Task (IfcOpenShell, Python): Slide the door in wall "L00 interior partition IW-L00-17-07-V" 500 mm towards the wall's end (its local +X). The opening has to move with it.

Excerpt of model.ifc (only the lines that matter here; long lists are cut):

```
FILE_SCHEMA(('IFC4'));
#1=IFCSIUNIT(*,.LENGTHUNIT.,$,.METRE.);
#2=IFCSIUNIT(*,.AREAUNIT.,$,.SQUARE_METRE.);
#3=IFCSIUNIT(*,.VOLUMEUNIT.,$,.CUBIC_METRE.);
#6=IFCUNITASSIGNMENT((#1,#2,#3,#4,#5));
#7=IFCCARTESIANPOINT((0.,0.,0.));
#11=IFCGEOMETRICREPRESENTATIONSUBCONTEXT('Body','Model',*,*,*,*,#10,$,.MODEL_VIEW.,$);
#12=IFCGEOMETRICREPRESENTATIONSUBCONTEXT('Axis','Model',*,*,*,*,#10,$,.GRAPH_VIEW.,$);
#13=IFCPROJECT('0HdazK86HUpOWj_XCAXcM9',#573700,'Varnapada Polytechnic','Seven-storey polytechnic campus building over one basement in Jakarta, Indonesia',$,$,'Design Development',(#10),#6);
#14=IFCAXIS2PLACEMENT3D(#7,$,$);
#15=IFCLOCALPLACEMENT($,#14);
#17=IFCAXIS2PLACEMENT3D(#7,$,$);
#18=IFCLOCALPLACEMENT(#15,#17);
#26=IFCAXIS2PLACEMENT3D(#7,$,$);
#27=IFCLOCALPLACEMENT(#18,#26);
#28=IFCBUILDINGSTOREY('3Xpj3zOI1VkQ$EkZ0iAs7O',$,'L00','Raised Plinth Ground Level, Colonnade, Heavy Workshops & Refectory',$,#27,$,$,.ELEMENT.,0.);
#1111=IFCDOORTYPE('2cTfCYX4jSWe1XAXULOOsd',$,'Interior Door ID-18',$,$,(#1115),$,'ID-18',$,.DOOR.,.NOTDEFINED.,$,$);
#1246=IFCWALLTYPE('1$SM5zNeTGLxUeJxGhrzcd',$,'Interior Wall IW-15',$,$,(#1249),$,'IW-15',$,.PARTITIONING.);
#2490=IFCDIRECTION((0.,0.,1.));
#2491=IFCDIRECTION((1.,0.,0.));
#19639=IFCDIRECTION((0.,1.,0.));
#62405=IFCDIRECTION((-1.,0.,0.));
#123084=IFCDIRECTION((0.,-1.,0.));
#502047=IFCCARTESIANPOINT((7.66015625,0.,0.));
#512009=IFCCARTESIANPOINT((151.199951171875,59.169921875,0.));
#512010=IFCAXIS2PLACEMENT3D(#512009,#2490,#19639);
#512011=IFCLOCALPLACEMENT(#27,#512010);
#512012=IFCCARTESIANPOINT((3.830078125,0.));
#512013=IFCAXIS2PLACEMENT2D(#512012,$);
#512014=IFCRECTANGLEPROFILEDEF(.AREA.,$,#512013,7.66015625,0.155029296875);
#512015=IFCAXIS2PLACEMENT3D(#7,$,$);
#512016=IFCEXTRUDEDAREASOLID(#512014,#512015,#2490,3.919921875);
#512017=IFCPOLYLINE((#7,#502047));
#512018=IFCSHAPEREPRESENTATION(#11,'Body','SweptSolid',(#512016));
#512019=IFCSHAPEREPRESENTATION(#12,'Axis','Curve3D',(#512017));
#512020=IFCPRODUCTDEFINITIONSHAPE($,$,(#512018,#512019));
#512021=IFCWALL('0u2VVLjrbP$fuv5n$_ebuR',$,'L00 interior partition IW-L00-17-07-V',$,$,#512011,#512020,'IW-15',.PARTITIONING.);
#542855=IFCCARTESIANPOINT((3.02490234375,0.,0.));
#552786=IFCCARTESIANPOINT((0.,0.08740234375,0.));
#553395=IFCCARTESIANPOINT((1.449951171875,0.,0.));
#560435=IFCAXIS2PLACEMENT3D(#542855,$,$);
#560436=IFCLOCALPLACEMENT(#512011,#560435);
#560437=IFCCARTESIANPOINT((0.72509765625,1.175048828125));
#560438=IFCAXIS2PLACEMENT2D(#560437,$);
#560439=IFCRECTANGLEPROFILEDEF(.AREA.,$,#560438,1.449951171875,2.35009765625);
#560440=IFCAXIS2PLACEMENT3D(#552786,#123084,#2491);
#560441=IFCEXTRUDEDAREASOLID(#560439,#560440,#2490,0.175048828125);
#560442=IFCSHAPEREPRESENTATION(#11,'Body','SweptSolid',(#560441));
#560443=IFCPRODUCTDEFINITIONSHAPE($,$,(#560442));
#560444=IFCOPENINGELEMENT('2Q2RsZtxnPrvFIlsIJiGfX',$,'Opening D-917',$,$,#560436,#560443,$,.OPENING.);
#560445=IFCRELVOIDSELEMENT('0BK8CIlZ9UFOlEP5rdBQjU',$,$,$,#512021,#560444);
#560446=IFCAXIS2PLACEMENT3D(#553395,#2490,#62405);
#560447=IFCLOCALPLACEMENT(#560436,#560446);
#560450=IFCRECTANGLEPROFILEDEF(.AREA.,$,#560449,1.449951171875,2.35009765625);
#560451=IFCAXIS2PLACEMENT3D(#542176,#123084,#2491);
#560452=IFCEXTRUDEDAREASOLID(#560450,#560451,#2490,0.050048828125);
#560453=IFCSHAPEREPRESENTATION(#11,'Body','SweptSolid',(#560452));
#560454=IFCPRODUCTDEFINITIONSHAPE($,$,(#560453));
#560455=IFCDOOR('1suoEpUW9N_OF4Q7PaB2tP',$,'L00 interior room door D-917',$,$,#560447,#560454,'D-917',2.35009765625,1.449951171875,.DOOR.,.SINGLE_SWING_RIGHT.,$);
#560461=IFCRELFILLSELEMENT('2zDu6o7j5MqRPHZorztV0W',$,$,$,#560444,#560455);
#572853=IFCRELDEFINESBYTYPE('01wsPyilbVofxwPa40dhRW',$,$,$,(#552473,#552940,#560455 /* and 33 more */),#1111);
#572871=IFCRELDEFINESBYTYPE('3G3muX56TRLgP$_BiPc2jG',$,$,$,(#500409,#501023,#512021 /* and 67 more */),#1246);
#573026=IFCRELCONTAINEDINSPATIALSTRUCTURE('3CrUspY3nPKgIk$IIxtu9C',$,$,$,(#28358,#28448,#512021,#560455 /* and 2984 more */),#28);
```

```python
import ifcopenshell
import ifcopenshell.api.geometry
import ifcopenshell.util.placement
import ifcopenshell.util.unit

model = ifcopenshell.open("model.ifc")
unit_scale = ifcopenshell.util.unit.calculate_unit_scale(model)

door = model.by_guid("1suoEpUW9N_OF4Q7PaB2tP")
opening = door.FillsVoids[0].RelatingOpeningElement
wall = opening.VoidsElements[0].RelatingBuildingElement

wall_matrix = ifcopenshell.util.placement.get_local_placement(wall.ObjectPlacement)
shift = wall_matrix[:3, 0] * 0.5 / unit_scale
before = ifcopenshell.util.placement.get_local_placement(door.ObjectPlacement)[:3, 3].copy()

# The door is placed relative to its opening, so it follows when the opening moves.
matrix = ifcopenshell.util.placement.get_local_placement(opening.ObjectPlacement)
matrix[:3, 3] += shift
ifcopenshell.api.geometry.edit_object_placement(
    model, product=opening, matrix=matrix, is_si=False, should_transform_children=True
)

after = ifcopenshell.util.placement.get_local_placement(door.ObjectPlacement)[:3, 3]
print("door moved by", (after - before).round(3) + 0.0)

model.write("model_v2.ifc")
```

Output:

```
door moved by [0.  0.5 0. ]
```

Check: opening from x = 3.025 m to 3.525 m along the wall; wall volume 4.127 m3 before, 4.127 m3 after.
